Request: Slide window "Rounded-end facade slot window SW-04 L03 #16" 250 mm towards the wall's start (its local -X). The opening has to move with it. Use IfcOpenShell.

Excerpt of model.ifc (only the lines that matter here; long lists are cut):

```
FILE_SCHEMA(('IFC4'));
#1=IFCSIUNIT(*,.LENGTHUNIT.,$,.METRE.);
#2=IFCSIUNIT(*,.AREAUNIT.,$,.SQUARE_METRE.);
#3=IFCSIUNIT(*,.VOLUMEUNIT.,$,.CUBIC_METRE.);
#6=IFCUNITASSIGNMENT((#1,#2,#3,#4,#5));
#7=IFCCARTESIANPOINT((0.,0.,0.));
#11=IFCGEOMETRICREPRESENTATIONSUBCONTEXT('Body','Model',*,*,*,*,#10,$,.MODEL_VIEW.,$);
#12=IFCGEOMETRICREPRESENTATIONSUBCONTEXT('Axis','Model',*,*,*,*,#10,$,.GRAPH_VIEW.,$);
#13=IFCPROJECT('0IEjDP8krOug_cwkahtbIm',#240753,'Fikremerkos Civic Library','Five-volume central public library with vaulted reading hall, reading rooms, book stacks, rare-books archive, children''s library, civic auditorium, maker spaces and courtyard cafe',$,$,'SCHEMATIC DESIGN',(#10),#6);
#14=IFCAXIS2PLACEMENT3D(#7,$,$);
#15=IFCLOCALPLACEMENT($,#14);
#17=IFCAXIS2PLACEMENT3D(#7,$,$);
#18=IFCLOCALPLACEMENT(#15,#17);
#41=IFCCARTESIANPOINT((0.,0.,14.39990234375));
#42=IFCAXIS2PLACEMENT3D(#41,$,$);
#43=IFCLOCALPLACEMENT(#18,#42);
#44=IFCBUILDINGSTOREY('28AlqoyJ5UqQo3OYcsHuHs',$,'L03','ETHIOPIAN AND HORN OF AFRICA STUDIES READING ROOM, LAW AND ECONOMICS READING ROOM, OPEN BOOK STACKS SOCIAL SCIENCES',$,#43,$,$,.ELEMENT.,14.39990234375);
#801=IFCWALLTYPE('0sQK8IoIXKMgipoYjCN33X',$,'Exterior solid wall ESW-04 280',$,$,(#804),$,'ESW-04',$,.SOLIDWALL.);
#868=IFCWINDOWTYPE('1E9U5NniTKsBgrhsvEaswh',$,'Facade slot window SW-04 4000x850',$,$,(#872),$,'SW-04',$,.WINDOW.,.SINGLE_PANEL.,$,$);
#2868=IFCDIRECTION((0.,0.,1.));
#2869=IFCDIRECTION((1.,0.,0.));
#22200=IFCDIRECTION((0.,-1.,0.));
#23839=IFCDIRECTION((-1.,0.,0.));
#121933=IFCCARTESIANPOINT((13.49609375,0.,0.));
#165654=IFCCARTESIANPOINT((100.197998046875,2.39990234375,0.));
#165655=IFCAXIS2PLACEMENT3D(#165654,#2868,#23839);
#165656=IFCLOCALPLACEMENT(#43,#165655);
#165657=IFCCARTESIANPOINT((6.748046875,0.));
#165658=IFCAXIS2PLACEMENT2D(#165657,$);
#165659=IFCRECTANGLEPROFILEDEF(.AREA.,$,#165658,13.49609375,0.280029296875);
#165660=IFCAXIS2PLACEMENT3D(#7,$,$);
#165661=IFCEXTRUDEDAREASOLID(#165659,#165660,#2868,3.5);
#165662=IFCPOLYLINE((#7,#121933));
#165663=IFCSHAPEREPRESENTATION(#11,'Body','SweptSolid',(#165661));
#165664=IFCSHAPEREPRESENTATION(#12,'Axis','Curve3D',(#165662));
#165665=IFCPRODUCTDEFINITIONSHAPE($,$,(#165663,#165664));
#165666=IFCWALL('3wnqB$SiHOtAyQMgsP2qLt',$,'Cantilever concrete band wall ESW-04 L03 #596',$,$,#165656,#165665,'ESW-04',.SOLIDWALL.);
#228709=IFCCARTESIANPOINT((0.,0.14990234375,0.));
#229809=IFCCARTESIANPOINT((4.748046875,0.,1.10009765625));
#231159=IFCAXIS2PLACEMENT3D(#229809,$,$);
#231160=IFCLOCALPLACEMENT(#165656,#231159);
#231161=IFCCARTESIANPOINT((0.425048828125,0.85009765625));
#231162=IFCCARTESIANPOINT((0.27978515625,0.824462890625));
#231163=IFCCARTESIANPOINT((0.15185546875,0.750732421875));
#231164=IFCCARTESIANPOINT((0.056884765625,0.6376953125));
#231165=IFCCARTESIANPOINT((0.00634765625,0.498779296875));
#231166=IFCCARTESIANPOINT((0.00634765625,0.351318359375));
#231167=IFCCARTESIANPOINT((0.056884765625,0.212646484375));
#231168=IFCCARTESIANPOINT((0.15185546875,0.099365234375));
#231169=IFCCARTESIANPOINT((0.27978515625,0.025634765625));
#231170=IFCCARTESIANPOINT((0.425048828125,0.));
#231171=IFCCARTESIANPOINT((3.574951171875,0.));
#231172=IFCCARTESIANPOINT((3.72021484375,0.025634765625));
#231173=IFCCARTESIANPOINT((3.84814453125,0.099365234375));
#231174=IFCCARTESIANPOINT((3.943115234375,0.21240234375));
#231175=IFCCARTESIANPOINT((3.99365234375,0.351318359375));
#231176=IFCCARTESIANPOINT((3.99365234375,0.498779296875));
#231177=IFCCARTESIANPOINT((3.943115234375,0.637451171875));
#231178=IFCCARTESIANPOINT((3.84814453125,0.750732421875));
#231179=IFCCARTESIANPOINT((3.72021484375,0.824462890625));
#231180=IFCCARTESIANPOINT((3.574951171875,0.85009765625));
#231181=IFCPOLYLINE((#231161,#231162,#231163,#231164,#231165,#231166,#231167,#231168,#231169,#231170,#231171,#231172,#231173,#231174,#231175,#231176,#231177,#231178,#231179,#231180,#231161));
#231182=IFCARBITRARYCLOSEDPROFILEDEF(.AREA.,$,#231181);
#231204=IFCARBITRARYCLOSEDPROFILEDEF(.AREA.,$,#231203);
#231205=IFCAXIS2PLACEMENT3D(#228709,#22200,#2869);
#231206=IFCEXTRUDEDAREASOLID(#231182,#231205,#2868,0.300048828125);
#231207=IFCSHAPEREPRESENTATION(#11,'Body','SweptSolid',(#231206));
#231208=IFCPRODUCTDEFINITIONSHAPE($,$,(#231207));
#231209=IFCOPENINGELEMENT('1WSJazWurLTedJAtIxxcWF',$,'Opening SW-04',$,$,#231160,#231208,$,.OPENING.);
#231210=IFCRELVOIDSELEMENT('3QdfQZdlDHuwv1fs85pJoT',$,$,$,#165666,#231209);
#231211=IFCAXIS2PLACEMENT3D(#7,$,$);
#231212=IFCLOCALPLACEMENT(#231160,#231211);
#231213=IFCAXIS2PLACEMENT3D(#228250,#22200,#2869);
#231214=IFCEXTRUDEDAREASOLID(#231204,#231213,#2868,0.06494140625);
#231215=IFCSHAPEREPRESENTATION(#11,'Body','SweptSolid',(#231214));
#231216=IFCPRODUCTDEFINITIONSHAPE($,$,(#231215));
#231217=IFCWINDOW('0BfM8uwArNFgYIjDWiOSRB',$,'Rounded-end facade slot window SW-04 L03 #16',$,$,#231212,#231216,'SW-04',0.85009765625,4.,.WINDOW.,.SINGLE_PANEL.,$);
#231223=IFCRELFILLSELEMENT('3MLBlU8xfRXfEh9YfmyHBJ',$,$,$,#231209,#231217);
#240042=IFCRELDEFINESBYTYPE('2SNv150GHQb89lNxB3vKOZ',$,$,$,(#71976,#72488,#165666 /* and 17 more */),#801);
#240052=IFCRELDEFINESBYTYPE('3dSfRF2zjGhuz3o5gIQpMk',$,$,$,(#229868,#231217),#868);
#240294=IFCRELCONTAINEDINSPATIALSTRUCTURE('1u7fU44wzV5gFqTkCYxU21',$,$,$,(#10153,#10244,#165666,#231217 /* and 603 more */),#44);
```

```python
import ifcopenshell
import ifcopenshell.api.geometry
import ifcopenshell.util.placement

model = ifcopenshell.open("model.ifc")

window = model.by_id(231217)
opening = window.FillsVoids[0].RelatingOpeningElement
wall = opening.VoidsElements[0].RelatingBuildingElement

wall_matrix = ifcopenshell.util.placement.get_local_placement(wall.ObjectPlacement)
shift = wall_matrix[:3, 0] * -0.25
before = ifcopenshell.util.placement.get_local_placement(window.ObjectPlacement)[:3, 3].copy()

# The window is placed relative to its opening, so it follows when the opening moves.
matrix = ifcopenshell.util.placement.get_local_placement(opening.ObjectPlacement)
matrix[:3, 3] += shift
ifcopenshell.api.geometry.edit_object_placement(
    model, product=opening, matrix=matrix, is_si=False, should_transform_children=True
)

after = ifcopenshell.util.placement.get_local_placement(window.ObjectPlacement)[:3, 3]
print("window moved by", (after - before).round(3) + 0.0)

model.write("model_updated.ifc")
```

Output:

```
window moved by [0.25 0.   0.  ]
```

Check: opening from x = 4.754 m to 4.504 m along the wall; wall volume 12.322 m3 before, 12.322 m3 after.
